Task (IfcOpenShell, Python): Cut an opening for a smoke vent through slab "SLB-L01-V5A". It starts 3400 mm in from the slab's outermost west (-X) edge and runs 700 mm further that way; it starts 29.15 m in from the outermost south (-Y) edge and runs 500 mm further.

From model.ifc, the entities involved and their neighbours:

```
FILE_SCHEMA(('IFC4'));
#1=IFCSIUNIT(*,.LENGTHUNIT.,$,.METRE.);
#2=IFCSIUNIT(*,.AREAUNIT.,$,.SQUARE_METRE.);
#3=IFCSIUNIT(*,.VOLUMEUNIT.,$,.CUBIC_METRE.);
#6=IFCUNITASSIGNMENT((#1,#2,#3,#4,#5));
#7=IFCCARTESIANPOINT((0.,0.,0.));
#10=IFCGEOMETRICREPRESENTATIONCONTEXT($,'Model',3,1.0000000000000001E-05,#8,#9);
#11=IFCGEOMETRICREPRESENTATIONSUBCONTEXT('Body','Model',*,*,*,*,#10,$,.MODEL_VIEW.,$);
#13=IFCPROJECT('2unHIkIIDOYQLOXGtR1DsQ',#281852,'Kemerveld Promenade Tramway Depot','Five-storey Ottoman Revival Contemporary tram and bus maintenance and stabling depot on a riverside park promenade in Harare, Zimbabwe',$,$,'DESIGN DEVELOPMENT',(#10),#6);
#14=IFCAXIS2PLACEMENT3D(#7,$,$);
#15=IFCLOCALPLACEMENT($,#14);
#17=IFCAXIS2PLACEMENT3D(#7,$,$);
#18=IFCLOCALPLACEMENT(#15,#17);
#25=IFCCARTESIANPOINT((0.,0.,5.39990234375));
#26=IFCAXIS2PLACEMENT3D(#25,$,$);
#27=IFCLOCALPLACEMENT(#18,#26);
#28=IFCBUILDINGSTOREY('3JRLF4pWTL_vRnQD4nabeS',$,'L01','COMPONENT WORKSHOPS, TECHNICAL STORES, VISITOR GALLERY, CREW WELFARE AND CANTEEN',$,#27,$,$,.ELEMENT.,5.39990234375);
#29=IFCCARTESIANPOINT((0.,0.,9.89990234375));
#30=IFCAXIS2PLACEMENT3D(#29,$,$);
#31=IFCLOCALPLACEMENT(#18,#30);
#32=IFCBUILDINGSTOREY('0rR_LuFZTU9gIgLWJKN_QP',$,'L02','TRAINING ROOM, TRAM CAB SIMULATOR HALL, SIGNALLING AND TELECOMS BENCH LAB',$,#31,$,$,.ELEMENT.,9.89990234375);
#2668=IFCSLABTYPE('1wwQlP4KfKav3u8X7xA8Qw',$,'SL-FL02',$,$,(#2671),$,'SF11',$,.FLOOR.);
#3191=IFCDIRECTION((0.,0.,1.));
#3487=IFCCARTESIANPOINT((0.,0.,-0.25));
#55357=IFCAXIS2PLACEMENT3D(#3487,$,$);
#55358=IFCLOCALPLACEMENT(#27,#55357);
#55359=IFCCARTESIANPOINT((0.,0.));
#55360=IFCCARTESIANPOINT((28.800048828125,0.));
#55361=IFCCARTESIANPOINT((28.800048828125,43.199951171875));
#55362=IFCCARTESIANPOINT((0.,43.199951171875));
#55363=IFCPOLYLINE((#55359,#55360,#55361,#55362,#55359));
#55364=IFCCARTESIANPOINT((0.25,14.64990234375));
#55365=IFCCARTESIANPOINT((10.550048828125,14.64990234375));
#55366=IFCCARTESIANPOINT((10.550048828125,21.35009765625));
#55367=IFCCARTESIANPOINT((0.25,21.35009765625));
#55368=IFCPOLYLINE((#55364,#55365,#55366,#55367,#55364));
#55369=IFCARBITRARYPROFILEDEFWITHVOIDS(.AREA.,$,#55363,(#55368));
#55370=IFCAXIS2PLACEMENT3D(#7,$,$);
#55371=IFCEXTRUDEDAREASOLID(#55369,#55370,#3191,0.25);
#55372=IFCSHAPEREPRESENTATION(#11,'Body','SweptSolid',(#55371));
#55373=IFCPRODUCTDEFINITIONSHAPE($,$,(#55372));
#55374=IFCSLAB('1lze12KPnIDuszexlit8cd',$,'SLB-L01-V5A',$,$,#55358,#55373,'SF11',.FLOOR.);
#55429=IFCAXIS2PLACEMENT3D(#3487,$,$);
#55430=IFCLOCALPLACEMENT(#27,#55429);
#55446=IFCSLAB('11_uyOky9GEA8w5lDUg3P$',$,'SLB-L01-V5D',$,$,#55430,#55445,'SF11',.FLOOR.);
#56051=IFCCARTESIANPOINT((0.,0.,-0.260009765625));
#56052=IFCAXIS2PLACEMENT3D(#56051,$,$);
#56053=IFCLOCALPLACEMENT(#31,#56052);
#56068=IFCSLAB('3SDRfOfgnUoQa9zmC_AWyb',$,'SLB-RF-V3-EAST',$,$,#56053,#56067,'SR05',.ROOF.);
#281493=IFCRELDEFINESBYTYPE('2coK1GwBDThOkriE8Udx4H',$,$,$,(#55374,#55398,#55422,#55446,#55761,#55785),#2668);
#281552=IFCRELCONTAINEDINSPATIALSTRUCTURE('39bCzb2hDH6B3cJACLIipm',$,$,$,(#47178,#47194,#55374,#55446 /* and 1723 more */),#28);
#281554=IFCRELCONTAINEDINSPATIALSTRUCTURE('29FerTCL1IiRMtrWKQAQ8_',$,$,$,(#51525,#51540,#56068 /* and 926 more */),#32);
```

```python
import numpy as np
import ifcopenshell
import ifcopenshell.api.feature
import ifcopenshell.api.geometry
import ifcopenshell.api.root
import ifcopenshell.geom
import ifcopenshell.util.placement
import ifcopenshell.util.representation
import ifcopenshell.util.shape
import ifcopenshell.util.unit

model = ifcopenshell.open("model.ifc")
unit_scale = ifcopenshell.util.unit.calculate_unit_scale(model)
settings = ifcopenshell.geom.settings()


def volume(element):
    """Net volume in cubic metres, openings subtracted."""
    shape = ifcopenshell.geom.create_shape(settings, element)
    return ifcopenshell.util.shape.get_volume(shape.geometry)


slab = model.by_guid("1lze12KPnIDuszexlit8cd")
before = volume(slab)

# Extent in the slab's own axes, in metres. The edges named are its -X and -Y sides.
slab_shape = ifcopenshell.geom.create_shape(settings, slab)
vertices = ifcopenshell.util.shape.get_vertices(slab_shape.geometry)
x_min, y_min, bottom = vertices.min(axis=0)
top = vertices[:, 2].max()

opening = ifcopenshell.api.root.create_entity(model, ifc_class="IfcOpeningElement", name="Smoke vent opening", predefined_type="OPENING")
context = ifcopenshell.util.representation.get_context(model, "Model", "Body", "MODEL_VIEW")
width, depth = 0.7, 0.5
outline = [(0.0, 0.0), (width, 0.0), (width, depth), (0.0, depth), (0.0, 0.0)]
# Overshoot both faces by 50 mm so the cut is clean.
shape = ifcopenshell.api.geometry.add_slab_representation(
    model, context=context, depth=top - bottom + 0.1, polyline=outline
)
ifcopenshell.api.geometry.assign_representation(model, product=opening, representation=shape)

matrix = ifcopenshell.util.placement.get_local_placement(slab.ObjectPlacement)
matrix[:, 3] = matrix @ np.append(np.array([x_min + 3.4, y_min + 29.15, bottom - 0.05]) / unit_scale, 1.0)
ifcopenshell.api.geometry.edit_object_placement(model, product=opening, matrix=matrix, is_si=False)
ifcopenshell.api.feature.add_feature(model, feature=opening, element=slab)

after = volume(slab)

print(f"slab volume {before:.3f} -> {after:.3f} m3")

model.write("model_v2.ifc")
```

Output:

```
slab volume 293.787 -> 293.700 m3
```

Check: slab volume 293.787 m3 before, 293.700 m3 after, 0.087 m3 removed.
